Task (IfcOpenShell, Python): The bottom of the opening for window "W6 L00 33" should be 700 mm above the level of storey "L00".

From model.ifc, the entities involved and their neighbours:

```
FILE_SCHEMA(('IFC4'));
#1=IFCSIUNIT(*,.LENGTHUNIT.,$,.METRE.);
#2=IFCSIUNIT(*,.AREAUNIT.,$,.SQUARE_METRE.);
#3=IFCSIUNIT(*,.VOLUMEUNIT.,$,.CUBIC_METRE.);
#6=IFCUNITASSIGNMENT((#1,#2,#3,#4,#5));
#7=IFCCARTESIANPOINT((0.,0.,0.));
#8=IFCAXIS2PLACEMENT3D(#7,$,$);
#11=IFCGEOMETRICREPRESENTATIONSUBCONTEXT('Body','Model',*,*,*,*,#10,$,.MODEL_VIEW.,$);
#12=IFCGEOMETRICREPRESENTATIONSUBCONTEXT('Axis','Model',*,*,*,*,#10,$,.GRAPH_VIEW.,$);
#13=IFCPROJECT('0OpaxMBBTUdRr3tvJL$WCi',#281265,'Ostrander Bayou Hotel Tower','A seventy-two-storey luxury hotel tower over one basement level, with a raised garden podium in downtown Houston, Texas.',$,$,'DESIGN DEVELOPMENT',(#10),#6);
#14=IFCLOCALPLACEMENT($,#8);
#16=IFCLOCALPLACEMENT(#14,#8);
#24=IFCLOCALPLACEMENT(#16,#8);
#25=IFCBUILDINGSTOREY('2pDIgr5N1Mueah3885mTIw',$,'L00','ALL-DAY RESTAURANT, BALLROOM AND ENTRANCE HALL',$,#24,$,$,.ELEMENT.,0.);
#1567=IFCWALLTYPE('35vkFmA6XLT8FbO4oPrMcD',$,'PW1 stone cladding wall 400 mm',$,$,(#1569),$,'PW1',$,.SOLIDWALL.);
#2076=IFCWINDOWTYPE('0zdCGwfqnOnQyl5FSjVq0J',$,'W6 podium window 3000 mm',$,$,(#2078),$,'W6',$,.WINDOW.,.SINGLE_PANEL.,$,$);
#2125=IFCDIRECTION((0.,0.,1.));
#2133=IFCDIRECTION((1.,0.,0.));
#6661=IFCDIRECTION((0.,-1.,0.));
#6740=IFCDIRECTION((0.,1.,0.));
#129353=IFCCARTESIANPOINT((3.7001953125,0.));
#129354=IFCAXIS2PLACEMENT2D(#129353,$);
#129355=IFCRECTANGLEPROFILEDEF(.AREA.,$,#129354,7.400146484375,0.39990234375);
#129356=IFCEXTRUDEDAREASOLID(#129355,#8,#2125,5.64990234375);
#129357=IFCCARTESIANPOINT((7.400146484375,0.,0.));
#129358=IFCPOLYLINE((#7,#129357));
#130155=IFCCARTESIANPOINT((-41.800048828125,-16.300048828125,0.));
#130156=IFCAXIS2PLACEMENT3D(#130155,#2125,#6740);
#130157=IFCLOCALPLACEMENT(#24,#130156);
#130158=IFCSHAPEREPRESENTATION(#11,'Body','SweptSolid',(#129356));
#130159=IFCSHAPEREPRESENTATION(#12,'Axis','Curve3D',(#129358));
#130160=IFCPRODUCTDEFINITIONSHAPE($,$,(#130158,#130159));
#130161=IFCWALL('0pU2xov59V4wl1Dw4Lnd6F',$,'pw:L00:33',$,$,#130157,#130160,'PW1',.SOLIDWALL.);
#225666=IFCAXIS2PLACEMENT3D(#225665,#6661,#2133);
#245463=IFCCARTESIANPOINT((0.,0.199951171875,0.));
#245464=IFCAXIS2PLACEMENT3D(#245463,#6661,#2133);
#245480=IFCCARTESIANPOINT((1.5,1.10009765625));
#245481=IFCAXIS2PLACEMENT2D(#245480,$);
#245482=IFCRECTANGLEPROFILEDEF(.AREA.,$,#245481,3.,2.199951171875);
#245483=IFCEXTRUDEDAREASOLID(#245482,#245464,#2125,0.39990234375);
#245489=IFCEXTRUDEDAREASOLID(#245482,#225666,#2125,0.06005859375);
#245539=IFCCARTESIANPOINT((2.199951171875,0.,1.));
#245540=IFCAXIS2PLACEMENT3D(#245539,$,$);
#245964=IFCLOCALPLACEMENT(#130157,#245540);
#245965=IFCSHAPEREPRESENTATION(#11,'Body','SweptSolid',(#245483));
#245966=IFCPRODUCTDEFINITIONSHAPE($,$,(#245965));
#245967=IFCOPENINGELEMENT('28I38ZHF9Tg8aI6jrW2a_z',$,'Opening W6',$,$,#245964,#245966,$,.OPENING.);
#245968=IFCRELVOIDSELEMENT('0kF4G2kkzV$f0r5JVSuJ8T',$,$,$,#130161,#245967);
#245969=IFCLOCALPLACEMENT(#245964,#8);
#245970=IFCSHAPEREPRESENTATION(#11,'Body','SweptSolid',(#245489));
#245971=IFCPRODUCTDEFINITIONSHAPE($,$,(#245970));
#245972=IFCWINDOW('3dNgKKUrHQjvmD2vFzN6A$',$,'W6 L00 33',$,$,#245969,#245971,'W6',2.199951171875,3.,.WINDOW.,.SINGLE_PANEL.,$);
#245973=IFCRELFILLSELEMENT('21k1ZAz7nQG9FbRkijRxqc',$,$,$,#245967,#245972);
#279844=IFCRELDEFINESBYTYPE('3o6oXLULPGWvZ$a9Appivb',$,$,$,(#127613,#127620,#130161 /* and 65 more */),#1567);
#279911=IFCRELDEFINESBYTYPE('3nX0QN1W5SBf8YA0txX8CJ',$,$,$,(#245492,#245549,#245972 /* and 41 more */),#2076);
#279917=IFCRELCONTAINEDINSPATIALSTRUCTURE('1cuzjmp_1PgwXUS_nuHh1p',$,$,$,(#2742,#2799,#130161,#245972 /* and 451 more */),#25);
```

```python
import numpy as np
import ifcopenshell
import ifcopenshell.api.geometry
import ifcopenshell.geom
import ifcopenshell.util.element
import ifcopenshell.util.placement
import ifcopenshell.util.shape
import ifcopenshell.util.unit

model = ifcopenshell.open("model.ifc")
unit_scale = ifcopenshell.util.unit.calculate_unit_scale(model)

window = model.by_guid("3dNgKKUrHQjvmD2vFzN6A$")
opening = window.FillsVoids[0].RelatingOpeningElement
storey = ifcopenshell.util.element.get_container(window, ifc_class="IfcBuildingStorey")
level = ifcopenshell.util.placement.get_local_placement(storey.ObjectPlacement)[2, 3]

# The opening's origin need not be at the sill, so measure its lowest point.
shape = ifcopenshell.geom.create_shape(ifcopenshell.geom.settings(), opening)
bottom = ifcopenshell.util.shape.get_shape_bottom_elevation(shape, shape.geometry) / unit_scale
dz = level + 0.7 - bottom

shift = np.array([0.0, 0.0, dz])
# The window is placed relative to its opening, so it follows when the opening moves.
matrix = ifcopenshell.util.placement.get_local_placement(opening.ObjectPlacement)
matrix[:3, 3] += shift
ifcopenshell.api.geometry.edit_object_placement(
    model, product=opening, matrix=matrix, is_si=False, should_transform_children=True
)

print(f"moved by {dz * unit_scale:+.3f} m")

model.write("model_rev.ifc")
```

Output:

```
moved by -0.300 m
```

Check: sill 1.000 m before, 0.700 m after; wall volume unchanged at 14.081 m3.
